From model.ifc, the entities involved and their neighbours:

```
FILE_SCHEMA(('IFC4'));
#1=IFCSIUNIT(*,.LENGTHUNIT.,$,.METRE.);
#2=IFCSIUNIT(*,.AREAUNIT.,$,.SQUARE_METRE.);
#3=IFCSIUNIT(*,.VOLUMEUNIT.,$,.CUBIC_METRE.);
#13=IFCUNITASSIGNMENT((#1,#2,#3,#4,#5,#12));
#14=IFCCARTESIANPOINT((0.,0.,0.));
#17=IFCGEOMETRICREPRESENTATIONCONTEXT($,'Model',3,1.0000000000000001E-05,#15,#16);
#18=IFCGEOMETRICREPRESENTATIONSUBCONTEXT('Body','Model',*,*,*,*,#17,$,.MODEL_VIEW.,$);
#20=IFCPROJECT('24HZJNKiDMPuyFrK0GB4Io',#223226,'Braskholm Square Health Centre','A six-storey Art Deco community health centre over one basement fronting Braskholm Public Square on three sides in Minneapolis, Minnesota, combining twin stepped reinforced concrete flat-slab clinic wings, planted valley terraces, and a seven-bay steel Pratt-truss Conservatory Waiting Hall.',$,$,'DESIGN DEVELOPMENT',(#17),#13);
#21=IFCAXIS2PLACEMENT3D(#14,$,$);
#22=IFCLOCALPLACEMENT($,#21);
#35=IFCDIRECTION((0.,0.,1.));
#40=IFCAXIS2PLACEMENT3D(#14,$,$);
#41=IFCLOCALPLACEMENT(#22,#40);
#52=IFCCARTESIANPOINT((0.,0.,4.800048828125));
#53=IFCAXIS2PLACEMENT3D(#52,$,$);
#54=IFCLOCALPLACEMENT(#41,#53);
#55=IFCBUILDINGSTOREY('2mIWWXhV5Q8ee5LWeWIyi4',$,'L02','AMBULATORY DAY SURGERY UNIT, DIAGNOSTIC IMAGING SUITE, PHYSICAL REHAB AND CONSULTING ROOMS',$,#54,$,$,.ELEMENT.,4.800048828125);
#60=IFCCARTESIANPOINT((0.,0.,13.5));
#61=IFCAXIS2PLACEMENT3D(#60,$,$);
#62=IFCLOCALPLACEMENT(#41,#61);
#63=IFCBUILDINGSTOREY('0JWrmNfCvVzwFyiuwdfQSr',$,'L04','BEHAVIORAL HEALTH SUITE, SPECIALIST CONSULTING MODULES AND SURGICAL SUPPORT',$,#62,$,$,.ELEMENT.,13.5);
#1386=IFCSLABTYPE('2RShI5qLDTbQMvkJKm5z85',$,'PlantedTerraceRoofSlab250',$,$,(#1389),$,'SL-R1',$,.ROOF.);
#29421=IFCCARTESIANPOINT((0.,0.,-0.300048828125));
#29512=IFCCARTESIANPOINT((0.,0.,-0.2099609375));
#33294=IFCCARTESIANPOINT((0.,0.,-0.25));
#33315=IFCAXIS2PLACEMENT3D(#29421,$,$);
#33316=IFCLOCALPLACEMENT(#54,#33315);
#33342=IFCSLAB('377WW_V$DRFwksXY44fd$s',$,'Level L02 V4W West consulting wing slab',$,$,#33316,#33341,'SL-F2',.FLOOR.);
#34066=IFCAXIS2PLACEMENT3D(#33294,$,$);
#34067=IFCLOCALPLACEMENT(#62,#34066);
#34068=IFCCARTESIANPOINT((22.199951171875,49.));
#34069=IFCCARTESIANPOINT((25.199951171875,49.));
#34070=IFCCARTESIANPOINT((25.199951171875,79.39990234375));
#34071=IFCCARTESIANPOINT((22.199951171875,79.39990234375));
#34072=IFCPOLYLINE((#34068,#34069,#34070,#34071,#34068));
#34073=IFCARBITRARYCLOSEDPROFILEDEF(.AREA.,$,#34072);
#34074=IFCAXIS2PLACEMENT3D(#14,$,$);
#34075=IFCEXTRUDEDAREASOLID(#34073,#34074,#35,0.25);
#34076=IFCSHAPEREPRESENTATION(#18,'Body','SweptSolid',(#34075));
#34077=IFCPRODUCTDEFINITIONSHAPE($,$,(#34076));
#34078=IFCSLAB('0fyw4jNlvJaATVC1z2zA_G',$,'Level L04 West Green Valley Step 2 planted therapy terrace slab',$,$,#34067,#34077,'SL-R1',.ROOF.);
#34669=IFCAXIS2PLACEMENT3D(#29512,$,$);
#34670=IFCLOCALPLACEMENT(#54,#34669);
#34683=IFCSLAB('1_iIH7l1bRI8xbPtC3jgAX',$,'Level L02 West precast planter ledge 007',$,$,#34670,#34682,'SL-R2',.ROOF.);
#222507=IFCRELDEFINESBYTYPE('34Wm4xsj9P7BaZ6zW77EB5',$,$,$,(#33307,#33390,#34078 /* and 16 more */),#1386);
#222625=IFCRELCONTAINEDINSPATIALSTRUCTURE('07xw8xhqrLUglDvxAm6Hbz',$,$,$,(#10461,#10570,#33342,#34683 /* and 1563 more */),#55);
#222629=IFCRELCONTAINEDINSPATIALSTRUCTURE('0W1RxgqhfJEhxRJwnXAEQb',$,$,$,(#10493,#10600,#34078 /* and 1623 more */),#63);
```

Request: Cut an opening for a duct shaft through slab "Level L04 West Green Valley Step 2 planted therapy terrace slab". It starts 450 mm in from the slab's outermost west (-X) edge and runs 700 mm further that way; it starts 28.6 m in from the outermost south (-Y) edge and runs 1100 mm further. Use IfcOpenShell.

```python
import numpy as np
import ifcopenshell
import ifcopenshell.api.feature
import ifcopenshell.api.geometry
import ifcopenshell.api.root
import ifcopenshell.geom
import ifcopenshell.util.placement
import ifcopenshell.util.representation
import ifcopenshell.util.shape
import ifcopenshell.util.unit

model = ifcopenshell.open("model.ifc")
unit_scale = ifcopenshell.util.unit.calculate_unit_scale(model)
settings = ifcopenshell.geom.settings()


def volume(element):
    """Net volume in cubic metres, openings subtracted."""
    shape = ifcopenshell.geom.create_shape(settings, element)
    return ifcopenshell.util.shape.get_volume(shape.geometry)


slab = model.by_id(34078)
before = volume(slab)

# Extent in the slab's own axes, in metres. The edges named are its -X and -Y sides.
slab_shape = ifcopenshell.geom.create_shape(settings, slab)
vertices = ifcopenshell.util.shape.get_vertices(slab_shape.geometry)
x_min, y_min, bottom = vertices.min(axis=0)
top = vertices[:, 2].max()

opening = ifcopenshell.api.root.create_entity(model, ifc_class="IfcOpeningElement", name="Duct shaft opening", predefined_type="OPENING")
context = ifcopenshell.util.representation.get_context(model, "Model", "Body", "MODEL_VIEW")
width, depth = 0.7, 1.1
outline = [(0.0, 0.0), (width, 0.0), (width, depth), (0.0, depth), (0.0, 0.0)]
# Overshoot both faces by 50 mm so the cut is clean.
shape = ifcopenshell.api.geometry.add_slab_representation(
    model, context=context, depth=top - bottom + 0.1, polyline=outline
)
ifcopenshell.api.geometry.assign_representation(model, product=opening, representation=shape)

matrix = ifcopenshell.util.placement.get_local_placement(slab.ObjectPlacement)
matrix[:, 3] = matrix @ np.append(np.array([x_min + 0.45, y_min + 28.6, bottom - 0.05]) / unit_scale, 1.0)
ifcopenshell.api.geometry.edit_object_placement(model, product=opening, matrix=matrix, is_si=False)
ifcopenshell.api.feature.add_feature(model, feature=opening, element=slab)

after = volume(slab)

print(f"slab volume {before:.3f} -> {after:.3f} m3")

model.write("model_v2.ifc")
```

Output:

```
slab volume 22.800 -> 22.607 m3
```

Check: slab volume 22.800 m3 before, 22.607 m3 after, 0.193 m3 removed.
